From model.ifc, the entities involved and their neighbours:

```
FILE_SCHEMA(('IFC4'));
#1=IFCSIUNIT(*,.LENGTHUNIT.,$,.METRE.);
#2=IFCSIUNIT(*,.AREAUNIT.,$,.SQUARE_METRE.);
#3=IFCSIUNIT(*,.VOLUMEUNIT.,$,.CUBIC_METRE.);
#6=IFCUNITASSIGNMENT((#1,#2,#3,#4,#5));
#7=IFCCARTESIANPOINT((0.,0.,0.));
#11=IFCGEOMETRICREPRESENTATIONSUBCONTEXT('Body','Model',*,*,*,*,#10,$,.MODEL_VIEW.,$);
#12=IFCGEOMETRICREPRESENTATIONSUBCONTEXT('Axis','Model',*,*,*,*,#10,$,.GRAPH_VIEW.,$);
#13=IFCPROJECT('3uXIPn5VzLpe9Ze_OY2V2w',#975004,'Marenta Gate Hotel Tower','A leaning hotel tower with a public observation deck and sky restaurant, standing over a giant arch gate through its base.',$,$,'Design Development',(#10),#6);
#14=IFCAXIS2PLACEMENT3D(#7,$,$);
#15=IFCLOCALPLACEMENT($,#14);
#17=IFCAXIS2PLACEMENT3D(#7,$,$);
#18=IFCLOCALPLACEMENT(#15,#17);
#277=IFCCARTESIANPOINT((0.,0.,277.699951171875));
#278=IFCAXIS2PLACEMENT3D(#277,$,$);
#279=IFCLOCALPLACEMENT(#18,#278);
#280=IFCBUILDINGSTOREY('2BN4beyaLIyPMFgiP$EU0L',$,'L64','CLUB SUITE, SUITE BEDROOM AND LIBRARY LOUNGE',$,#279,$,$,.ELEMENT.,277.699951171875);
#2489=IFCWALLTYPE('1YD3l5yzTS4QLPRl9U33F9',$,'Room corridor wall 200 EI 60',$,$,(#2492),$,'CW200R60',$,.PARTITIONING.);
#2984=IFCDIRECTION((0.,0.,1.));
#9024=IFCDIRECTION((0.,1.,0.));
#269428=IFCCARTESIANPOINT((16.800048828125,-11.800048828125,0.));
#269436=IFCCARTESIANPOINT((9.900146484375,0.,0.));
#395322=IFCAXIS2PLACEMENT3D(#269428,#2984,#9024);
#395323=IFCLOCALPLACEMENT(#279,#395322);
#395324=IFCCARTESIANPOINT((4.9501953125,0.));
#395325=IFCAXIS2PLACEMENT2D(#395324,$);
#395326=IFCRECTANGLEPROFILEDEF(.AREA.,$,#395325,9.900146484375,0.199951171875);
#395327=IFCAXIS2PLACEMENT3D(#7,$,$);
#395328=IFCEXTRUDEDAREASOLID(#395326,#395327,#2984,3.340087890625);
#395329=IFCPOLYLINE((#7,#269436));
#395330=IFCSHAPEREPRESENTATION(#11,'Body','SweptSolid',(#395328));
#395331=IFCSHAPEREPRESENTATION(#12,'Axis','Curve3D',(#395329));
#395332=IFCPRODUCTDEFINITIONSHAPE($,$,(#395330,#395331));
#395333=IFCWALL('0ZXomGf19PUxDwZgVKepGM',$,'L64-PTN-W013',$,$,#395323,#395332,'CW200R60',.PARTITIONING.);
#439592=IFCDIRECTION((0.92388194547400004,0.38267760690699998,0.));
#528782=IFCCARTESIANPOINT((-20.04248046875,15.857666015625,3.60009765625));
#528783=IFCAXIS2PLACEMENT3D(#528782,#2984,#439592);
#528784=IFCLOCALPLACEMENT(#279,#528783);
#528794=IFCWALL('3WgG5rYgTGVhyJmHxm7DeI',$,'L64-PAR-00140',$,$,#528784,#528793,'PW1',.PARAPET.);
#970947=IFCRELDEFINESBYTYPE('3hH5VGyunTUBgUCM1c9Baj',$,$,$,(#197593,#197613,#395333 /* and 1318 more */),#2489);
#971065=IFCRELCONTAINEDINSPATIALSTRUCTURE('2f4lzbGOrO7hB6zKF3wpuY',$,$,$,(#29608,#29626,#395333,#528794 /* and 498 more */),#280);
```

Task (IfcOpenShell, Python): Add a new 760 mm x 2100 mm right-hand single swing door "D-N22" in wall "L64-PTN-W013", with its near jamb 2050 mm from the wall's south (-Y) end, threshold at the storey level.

```python
import numpy as np
import ifcopenshell
import ifcopenshell.api.feature
import ifcopenshell.api.geometry
import ifcopenshell.api.root
import ifcopenshell.api.spatial
import ifcopenshell.geom
import ifcopenshell.util.element
import ifcopenshell.util.placement
import ifcopenshell.util.representation
import ifcopenshell.util.shape
import ifcopenshell.util.unit

model = ifcopenshell.open("model.ifc")
unit_scale = ifcopenshell.util.unit.calculate_unit_scale(model)
settings = ifcopenshell.geom.settings()


def volume(element):
    """Net volume in cubic metres, openings subtracted."""
    shape = ifcopenshell.geom.create_shape(settings, element)
    return ifcopenshell.util.shape.get_volume(shape.geometry)


wall = model.by_id(395333)
storey = ifcopenshell.util.element.get_container(wall, ifc_class="IfcBuildingStorey")
context = ifcopenshell.util.representation.get_context(model, "Model", "Body", "MODEL_VIEW")
before = volume(wall)

width, height, from_end, sill = 0.76, 2.1, 2.05, 0.0  # metres

# The wall runs along its own X axis, and the end named is its -X end.
wall_shape = ifcopenshell.geom.create_shape(settings, wall)
x, y, z = ifcopenshell.util.shape.get_vertices(wall_shape.geometry).T
start = x.min() + from_end
face, thickness = float(y.min()), float(y.max() - y.min())
wall_matrix = ifcopenshell.util.placement.get_local_placement(wall.ObjectPlacement)
level = ifcopenshell.util.placement.get_local_placement(storey.ObjectPlacement)[2, 3]


def in_wall(x, y):
    """Placement at x, y metres in the wall's axes, at sill height."""
    matrix = wall_matrix.copy()
    matrix[:, 3] = wall_matrix @ np.array([x / unit_scale, y / unit_scale, 0.0, 1.0])
    matrix[2, 3] = level + sill / unit_scale
    return matrix


# Opening: a box that overshoots both wall faces by 50 mm.
opening = ifcopenshell.api.root.create_entity(model, ifc_class="IfcOpeningElement", predefined_type="OPENING")
box = ifcopenshell.api.geometry.add_wall_representation(
    model, context=context, length=width, height=height, thickness=thickness + 0.1
)
ifcopenshell.api.geometry.assign_representation(model, product=opening, representation=box)
ifcopenshell.api.geometry.edit_object_placement(model, product=opening, matrix=in_wall(start, face - 0.05), is_si=False)
ifcopenshell.api.feature.add_feature(model, feature=opening, element=wall)

door = ifcopenshell.api.root.create_entity(model, ifc_class="IfcDoor", name="D-N22", predefined_type="DOOR")
door.OverallWidth, door.OverallHeight = width / unit_scale, height / unit_scale
door.OperationType = "SINGLE_SWING_RIGHT"
body = ifcopenshell.api.geometry.add_door_representation(
    model,
    context=context,
    overall_width=door.OverallWidth,
    overall_height=door.OverallHeight,
    operation_type="SINGLE_SWING_RIGHT",
    lining_properties={"LiningDepth": thickness / unit_scale, "ThresholdDepth": thickness / unit_scale},
)
ifcopenshell.api.geometry.assign_representation(model, product=door, representation=body)
ifcopenshell.api.spatial.assign_container(model, products=[door], relating_structure=storey)
ifcopenshell.api.feature.add_filling(model, opening=opening, element=door)

# The lining spans the wall, so the door starts at the wall face.
ifcopenshell.api.geometry.edit_object_placement(model, product=door, matrix=in_wall(start, face), is_si=False)

after = volume(wall)

print(f"wall volume {before:.3f} -> {after:.3f} m3")

model.write("model_rev.ifc")
```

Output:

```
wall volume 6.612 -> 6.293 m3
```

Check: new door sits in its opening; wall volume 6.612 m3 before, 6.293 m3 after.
